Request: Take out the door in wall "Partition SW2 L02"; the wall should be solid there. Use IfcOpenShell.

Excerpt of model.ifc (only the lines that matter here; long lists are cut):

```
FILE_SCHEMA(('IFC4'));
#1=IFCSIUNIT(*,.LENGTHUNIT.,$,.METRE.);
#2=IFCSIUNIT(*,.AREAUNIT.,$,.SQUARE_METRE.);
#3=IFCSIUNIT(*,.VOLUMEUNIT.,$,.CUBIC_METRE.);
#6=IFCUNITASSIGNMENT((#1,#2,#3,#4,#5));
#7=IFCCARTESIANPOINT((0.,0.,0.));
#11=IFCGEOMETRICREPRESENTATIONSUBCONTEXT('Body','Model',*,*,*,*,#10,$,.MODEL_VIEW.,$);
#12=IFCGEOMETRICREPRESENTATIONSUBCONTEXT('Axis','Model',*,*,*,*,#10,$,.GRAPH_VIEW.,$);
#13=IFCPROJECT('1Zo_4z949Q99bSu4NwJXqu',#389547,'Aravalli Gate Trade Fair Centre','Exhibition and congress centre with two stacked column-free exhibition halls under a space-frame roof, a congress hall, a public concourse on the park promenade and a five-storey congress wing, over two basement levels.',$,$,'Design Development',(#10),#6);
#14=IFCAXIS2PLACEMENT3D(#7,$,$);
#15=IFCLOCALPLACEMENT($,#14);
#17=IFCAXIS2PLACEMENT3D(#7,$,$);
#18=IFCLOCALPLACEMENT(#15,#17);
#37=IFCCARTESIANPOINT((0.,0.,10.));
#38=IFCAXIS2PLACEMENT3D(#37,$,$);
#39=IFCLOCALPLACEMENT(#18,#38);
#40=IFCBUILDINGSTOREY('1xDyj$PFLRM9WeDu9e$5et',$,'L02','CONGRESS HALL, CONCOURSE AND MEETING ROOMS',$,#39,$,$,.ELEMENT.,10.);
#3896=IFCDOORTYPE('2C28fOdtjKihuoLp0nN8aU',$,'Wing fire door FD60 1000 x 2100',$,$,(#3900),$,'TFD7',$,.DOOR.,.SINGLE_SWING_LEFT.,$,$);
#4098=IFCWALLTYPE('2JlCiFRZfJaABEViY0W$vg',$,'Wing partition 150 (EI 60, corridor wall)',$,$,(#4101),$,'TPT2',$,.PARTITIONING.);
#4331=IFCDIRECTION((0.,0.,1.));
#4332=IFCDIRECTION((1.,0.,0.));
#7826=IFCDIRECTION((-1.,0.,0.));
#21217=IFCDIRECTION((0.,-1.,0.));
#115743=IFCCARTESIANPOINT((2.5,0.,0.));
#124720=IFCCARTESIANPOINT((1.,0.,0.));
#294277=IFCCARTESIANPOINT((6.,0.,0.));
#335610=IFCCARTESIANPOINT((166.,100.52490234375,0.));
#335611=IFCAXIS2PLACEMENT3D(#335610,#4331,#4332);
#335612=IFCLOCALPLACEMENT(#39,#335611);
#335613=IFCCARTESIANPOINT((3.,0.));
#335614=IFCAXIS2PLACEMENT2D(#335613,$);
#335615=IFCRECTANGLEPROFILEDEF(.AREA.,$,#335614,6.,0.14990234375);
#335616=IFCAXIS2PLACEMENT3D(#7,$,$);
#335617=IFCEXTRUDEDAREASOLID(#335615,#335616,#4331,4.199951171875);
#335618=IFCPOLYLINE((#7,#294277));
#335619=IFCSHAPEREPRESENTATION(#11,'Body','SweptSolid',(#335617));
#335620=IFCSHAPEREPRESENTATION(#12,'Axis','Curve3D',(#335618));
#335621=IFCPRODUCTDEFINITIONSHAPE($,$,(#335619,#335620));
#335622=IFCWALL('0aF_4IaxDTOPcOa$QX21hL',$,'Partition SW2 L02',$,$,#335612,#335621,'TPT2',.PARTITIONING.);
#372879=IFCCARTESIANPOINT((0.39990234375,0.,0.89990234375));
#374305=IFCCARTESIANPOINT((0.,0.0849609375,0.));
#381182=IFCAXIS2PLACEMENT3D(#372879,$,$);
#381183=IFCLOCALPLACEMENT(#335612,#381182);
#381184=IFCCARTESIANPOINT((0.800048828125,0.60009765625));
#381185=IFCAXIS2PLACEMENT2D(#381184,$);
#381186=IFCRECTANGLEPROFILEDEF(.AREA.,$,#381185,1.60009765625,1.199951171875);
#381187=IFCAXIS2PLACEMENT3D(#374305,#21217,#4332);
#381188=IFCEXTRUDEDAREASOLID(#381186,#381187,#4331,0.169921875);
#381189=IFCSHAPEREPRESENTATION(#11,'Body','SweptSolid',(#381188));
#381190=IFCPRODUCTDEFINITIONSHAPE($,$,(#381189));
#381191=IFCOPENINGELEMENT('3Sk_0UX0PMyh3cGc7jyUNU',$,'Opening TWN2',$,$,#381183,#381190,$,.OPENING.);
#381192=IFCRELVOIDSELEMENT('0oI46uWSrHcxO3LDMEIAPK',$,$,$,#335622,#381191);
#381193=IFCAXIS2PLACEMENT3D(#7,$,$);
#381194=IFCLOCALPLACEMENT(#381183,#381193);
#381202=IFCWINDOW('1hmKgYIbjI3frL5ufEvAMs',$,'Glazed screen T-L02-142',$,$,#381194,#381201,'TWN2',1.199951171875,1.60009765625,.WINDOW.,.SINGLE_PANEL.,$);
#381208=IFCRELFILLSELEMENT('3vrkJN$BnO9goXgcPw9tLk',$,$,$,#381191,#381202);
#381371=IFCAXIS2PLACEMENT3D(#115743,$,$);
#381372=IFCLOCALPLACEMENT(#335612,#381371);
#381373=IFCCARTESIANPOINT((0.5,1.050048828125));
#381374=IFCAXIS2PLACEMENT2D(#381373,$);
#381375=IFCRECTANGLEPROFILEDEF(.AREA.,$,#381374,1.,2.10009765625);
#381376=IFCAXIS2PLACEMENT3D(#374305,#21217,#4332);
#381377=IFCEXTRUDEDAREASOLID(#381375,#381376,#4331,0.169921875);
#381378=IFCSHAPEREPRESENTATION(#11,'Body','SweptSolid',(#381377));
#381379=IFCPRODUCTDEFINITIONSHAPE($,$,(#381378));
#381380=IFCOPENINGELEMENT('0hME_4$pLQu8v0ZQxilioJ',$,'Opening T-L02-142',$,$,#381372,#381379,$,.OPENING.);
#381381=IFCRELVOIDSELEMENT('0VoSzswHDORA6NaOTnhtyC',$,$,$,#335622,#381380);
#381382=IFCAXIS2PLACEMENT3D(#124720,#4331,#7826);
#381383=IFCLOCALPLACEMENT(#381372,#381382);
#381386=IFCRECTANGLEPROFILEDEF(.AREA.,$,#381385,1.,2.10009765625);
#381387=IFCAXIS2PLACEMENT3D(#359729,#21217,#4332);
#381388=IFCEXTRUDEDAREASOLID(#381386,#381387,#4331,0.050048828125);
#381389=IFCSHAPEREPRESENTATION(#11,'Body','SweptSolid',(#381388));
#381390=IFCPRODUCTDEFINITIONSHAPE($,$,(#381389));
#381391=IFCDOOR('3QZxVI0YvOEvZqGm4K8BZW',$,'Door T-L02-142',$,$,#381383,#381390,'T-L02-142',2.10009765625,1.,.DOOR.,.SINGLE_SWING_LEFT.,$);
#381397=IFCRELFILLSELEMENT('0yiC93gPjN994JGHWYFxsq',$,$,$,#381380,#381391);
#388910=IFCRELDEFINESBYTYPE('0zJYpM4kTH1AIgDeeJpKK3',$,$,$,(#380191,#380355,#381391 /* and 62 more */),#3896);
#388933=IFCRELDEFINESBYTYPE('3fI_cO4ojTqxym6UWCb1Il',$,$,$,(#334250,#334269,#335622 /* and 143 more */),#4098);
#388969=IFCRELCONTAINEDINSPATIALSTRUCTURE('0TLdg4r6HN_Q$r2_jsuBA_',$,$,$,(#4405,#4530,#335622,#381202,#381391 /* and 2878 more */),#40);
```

```python
import ifcopenshell
import ifcopenshell.api.feature
import ifcopenshell.api.root
import ifcopenshell.geom
import ifcopenshell.util.shape

model = ifcopenshell.open("model.ifc")
settings = ifcopenshell.geom.settings()


def volume(element):
    """Net volume in cubic metres, openings subtracted."""
    shape = ifcopenshell.geom.create_shape(settings, element)
    return ifcopenshell.util.shape.get_volume(shape.geometry)


door = model.by_guid("3QZxVI0YvOEvZqGm4K8BZW")
opening = door.FillsVoids[0].RelatingOpeningElement
wall = opening.VoidsElements[0].RelatingBuildingElement
before = volume(wall)

ifcopenshell.api.root.remove_product(model, product=door)
ifcopenshell.api.feature.remove_feature(model, feature=opening)

after = volume(wall)

print(f"wall volume {before:.3f} -> {after:.3f} m3")

model.write("model_edited.ifc")
```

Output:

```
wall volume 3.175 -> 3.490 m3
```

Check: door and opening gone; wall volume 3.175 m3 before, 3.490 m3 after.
